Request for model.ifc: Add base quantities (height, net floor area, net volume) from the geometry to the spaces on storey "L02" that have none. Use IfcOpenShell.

First a look at what the model holds.

```python
import ifcopenshell
import ifcopenshell.util.element
import ifcopenshell.util.unit

model = ifcopenshell.open("model.ifc")
print(model.schema)
for unit_type in ("LENGTHUNIT", "AREAUNIT", "VOLUMEUNIT"):
    print(unit_type, ifcopenshell.util.unit.calculate_unit_scale(model, unit_type))
storey = next(s for s in model.by_type("IfcBuildingStorey") if s.Name == "L02")
spaces = [e for e in ifcopenshell.util.element.get_decomposition(storey) if e.is_a("IfcSpace")]
for e in sorted(spaces, key=lambda e: e.id()):
    print(e.id(), e.is_a(), e.Name, list(ifcopenshell.util.element.get_psets(e, qtos_only=True)), sep=" | ")
```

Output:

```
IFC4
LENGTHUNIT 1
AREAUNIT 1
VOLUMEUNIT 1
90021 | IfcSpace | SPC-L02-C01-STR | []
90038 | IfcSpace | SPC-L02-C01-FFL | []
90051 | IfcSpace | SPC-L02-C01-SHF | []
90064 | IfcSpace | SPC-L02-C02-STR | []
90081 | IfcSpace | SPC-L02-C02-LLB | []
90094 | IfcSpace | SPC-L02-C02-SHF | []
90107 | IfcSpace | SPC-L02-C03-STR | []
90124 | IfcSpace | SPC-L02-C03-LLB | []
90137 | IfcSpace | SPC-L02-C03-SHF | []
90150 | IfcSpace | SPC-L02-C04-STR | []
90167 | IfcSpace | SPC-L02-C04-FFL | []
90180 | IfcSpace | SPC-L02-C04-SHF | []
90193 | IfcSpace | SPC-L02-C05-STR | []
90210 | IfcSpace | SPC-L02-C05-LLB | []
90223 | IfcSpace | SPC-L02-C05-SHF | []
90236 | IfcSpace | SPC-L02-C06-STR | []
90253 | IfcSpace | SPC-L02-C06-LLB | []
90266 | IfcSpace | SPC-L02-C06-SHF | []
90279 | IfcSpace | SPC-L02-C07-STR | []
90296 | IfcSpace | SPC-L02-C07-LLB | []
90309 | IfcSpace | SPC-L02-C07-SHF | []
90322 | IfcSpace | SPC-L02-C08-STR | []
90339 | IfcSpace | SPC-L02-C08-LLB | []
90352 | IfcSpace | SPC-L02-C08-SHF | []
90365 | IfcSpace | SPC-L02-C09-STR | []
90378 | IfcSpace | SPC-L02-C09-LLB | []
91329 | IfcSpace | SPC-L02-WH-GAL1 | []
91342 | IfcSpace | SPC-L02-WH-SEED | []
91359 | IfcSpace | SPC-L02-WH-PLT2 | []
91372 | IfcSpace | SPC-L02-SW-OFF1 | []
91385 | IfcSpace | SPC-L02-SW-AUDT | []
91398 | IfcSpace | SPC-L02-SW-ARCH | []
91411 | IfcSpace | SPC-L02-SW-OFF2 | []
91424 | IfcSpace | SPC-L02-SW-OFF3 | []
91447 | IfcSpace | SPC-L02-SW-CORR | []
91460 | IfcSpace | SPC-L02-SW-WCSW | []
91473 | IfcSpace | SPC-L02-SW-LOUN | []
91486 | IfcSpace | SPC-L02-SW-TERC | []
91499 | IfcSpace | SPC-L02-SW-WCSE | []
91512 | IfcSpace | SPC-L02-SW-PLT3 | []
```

```python
import ifcopenshell
import ifcopenshell.api.pset
import ifcopenshell.geom
import ifcopenshell.util.element
import ifcopenshell.util.shape
import ifcopenshell.util.unit

model = ifcopenshell.open("model.ifc")
unit_scale = ifcopenshell.util.unit.calculate_unit_scale(model)
area_scale = ifcopenshell.util.unit.calculate_unit_scale(model, "AREAUNIT")
volume_scale = ifcopenshell.util.unit.calculate_unit_scale(model, "VOLUMEUNIT")
settings = ifcopenshell.geom.settings()

storey = next(s for s in model.by_type("IfcBuildingStorey") if s.Name == "L02")
spaces = [e for e in ifcopenshell.util.element.get_decomposition(storey) if e.is_a("IfcSpace")]

for e in sorted(spaces, key=lambda e: e.id()):
    if ifcopenshell.util.element.get_psets(e, qtos_only=True, should_inherit=False):
        continue
    # Geometry comes back in metres, in the element's own axes.
    shape = ifcopenshell.geom.create_shape(settings, e)
    values = {
        "Height": ifcopenshell.util.shape.get_z(shape.geometry) / unit_scale,
        "NetFloorArea": ifcopenshell.util.shape.get_footprint_area(shape.geometry) / area_scale,
        "NetVolume": ifcopenshell.util.shape.get_volume(shape.geometry) / volume_scale,
    }
    qto = ifcopenshell.api.pset.add_qto(model, product=e, name="Qto_SpaceBaseQuantities")
    ifcopenshell.api.pset.edit_qto(model, qto=qto, properties=values)
    print(e.id(), {k: round(v, 3) for k, v in values.items()})

model.write("model_rev.ifc")
```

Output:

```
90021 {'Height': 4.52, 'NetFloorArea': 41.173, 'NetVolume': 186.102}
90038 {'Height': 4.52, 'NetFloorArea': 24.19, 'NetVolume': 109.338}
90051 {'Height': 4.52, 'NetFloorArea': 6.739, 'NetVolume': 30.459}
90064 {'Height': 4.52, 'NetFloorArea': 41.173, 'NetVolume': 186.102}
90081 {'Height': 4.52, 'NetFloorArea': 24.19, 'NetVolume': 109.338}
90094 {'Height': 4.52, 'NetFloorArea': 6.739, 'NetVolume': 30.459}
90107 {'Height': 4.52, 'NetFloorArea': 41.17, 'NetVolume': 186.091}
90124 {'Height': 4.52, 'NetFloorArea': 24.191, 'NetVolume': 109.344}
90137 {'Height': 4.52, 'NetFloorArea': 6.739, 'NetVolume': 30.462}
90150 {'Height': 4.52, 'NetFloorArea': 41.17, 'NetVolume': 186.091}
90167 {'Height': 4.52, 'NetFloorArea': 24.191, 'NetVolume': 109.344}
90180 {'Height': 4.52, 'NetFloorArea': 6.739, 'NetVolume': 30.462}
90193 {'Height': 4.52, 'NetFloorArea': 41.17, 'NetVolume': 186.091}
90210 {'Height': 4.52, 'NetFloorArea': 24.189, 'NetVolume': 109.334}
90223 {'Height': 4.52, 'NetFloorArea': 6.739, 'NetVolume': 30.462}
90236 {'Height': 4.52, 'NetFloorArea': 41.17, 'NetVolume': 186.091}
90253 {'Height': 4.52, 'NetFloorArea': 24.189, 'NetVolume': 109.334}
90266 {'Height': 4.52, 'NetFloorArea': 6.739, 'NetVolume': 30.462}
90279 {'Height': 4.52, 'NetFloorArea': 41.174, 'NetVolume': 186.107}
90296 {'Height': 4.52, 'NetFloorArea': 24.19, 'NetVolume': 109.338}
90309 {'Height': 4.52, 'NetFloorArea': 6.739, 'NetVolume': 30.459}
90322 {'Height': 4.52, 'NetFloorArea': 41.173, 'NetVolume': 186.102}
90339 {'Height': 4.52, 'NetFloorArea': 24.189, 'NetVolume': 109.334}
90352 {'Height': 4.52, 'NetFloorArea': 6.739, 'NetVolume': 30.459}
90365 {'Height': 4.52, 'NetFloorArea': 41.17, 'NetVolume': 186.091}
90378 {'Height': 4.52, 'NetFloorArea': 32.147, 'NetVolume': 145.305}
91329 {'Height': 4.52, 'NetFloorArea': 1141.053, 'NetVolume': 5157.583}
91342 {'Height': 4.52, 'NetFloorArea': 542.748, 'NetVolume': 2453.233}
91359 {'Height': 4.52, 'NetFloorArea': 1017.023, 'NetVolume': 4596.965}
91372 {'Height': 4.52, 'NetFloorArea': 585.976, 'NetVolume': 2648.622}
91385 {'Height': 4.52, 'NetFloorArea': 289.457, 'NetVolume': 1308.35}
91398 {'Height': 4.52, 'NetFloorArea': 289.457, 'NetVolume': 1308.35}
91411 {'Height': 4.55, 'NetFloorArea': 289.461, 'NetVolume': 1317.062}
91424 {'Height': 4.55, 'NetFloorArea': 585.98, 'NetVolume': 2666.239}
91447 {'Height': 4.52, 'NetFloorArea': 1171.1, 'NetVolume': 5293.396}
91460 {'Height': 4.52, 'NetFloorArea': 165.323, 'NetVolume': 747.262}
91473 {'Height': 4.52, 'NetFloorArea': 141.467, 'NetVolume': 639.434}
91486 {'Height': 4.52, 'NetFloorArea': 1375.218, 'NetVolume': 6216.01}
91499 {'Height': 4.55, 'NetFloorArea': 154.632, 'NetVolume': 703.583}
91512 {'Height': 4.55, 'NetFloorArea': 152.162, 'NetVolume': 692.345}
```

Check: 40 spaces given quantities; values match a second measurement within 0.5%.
